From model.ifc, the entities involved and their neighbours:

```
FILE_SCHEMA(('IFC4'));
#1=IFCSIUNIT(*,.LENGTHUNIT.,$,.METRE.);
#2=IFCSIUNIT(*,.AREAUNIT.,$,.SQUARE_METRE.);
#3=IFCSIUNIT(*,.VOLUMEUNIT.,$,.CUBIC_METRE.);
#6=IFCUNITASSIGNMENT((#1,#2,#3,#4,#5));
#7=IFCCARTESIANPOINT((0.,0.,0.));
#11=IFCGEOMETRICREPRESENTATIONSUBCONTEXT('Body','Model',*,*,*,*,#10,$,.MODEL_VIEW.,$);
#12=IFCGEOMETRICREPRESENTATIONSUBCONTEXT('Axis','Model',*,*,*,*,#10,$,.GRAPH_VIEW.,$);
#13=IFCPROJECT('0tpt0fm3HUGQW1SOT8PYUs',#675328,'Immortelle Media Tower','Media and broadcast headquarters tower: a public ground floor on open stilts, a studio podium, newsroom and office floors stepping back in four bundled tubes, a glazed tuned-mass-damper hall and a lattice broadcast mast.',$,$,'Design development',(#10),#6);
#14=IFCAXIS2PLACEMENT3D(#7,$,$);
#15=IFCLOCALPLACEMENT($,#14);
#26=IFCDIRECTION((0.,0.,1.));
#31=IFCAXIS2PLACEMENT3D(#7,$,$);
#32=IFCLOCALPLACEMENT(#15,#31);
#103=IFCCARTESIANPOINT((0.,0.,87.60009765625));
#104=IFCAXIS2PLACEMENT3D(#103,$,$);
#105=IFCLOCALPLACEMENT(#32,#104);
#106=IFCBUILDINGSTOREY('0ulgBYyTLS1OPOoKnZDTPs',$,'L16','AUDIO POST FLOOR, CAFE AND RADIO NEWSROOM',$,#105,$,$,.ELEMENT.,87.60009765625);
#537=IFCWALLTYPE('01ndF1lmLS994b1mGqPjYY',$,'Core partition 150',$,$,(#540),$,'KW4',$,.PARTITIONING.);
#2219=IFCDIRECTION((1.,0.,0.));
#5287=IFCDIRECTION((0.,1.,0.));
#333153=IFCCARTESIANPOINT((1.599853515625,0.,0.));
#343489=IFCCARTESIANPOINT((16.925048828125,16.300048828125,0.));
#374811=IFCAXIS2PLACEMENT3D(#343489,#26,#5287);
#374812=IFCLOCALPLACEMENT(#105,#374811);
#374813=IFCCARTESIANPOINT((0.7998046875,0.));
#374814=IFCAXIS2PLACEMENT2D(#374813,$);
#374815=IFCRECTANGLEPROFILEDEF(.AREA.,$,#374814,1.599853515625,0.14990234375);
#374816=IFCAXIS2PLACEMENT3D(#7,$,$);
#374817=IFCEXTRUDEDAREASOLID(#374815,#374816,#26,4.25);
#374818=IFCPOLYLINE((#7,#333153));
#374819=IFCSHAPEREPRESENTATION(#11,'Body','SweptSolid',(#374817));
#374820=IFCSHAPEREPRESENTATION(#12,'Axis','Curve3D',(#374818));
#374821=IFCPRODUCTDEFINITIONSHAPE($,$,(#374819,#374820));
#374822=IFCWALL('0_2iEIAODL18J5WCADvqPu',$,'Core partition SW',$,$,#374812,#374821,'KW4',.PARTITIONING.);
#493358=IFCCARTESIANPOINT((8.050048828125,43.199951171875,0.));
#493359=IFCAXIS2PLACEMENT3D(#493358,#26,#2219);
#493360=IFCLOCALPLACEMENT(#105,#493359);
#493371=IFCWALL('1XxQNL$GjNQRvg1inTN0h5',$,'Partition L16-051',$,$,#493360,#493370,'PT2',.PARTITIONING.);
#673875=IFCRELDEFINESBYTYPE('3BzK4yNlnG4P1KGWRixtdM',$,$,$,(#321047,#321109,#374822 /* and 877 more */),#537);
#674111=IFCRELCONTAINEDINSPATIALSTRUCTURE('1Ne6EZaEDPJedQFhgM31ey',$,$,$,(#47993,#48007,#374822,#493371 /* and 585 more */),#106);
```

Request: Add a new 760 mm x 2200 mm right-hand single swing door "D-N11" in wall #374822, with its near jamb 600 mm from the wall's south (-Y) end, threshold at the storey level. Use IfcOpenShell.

```python
import numpy as np
import ifcopenshell
import ifcopenshell.api.feature
import ifcopenshell.api.geometry
import ifcopenshell.api.root
import ifcopenshell.api.spatial
import ifcopenshell.geom
import ifcopenshell.util.element
import ifcopenshell.util.placement
import ifcopenshell.util.representation
import ifcopenshell.util.shape
import ifcopenshell.util.unit

model = ifcopenshell.open("model.ifc")
unit_scale = ifcopenshell.util.unit.calculate_unit_scale(model)
settings = ifcopenshell.geom.settings()


def volume(element):
    """Net volume in cubic metres, openings subtracted."""
    shape = ifcopenshell.geom.create_shape(settings, element)
    return ifcopenshell.util.shape.get_volume(shape.geometry)


wall = model.by_guid("0_2iEIAODL18J5WCADvqPu")
storey = ifcopenshell.util.element.get_container(wall, ifc_class="IfcBuildingStorey")
context = ifcopenshell.util.representation.get_context(model, "Model", "Body", "MODEL_VIEW")
before = volume(wall)

width, height, from_end, sill = 0.76, 2.2, 0.6, 0.0  # metres

# The wall runs along its own X axis, and the end named is its -X end.
wall_shape = ifcopenshell.geom.create_shape(settings, wall)
x, y, z = ifcopenshell.util.shape.get_vertices(wall_shape.geometry).T
start = x.min() + from_end
face, thickness = float(y.min()), float(y.max() - y.min())
wall_matrix = ifcopenshell.util.placement.get_local_placement(wall.ObjectPlacement)
level = ifcopenshell.util.placement.get_local_placement(storey.ObjectPlacement)[2, 3]


def in_wall(x, y):
    """Placement at x, y metres in the wall's axes, at sill height."""
    matrix = wall_matrix.copy()
    matrix[:, 3] = wall_matrix @ np.array([x / unit_scale, y / unit_scale, 0.0, 1.0])
    matrix[2, 3] = level + sill / unit_scale
    return matrix


# Opening: a box that overshoots both wall faces by 50 mm.
opening = ifcopenshell.api.root.create_entity(model, ifc_class="IfcOpeningElement", predefined_type="OPENING")
box = ifcopenshell.api.geometry.add_wall_representation(
    model, context=context, length=width, height=height, thickness=thickness + 0.1
)
ifcopenshell.api.geometry.assign_representation(model, product=opening, representation=box)
ifcopenshell.api.geometry.edit_object_placement(model, product=opening, matrix=in_wall(start, face - 0.05), is_si=False)
ifcopenshell.api.feature.add_feature(model, feature=opening, element=wall)

door = ifcopenshell.api.root.create_entity(model, ifc_class="IfcDoor", name="D-N11", predefined_type="DOOR")
door.OverallWidth, door.OverallHeight = width / unit_scale, height / unit_scale
door.OperationType = "SINGLE_SWING_RIGHT"
body = ifcopenshell.api.geometry.add_door_representation(
    model,
    context=context,
    overall_width=door.OverallWidth,
    overall_height=door.OverallHeight,
    operation_type="SINGLE_SWING_RIGHT",
    lining_properties={"LiningDepth": thickness / unit_scale, "ThresholdDepth": thickness / unit_scale},
)
ifcopenshell.api.geometry.assign_representation(model, product=door, representation=body)
ifcopenshell.api.spatial.assign_container(model, products=[door], relating_structure=storey)
ifcopenshell.api.feature.add_filling(model, opening=opening, element=door)

# The lining spans the wall, so the door starts at the wall face.
ifcopenshell.api.geometry.edit_object_placement(model, product=door, matrix=in_wall(start, face), is_si=False)

after = volume(wall)

print(f"wall volume {before:.3f} -> {after:.3f} m3")

model.write("model_v2.ifc")
```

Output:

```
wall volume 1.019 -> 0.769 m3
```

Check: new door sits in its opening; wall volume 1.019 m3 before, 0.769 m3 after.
